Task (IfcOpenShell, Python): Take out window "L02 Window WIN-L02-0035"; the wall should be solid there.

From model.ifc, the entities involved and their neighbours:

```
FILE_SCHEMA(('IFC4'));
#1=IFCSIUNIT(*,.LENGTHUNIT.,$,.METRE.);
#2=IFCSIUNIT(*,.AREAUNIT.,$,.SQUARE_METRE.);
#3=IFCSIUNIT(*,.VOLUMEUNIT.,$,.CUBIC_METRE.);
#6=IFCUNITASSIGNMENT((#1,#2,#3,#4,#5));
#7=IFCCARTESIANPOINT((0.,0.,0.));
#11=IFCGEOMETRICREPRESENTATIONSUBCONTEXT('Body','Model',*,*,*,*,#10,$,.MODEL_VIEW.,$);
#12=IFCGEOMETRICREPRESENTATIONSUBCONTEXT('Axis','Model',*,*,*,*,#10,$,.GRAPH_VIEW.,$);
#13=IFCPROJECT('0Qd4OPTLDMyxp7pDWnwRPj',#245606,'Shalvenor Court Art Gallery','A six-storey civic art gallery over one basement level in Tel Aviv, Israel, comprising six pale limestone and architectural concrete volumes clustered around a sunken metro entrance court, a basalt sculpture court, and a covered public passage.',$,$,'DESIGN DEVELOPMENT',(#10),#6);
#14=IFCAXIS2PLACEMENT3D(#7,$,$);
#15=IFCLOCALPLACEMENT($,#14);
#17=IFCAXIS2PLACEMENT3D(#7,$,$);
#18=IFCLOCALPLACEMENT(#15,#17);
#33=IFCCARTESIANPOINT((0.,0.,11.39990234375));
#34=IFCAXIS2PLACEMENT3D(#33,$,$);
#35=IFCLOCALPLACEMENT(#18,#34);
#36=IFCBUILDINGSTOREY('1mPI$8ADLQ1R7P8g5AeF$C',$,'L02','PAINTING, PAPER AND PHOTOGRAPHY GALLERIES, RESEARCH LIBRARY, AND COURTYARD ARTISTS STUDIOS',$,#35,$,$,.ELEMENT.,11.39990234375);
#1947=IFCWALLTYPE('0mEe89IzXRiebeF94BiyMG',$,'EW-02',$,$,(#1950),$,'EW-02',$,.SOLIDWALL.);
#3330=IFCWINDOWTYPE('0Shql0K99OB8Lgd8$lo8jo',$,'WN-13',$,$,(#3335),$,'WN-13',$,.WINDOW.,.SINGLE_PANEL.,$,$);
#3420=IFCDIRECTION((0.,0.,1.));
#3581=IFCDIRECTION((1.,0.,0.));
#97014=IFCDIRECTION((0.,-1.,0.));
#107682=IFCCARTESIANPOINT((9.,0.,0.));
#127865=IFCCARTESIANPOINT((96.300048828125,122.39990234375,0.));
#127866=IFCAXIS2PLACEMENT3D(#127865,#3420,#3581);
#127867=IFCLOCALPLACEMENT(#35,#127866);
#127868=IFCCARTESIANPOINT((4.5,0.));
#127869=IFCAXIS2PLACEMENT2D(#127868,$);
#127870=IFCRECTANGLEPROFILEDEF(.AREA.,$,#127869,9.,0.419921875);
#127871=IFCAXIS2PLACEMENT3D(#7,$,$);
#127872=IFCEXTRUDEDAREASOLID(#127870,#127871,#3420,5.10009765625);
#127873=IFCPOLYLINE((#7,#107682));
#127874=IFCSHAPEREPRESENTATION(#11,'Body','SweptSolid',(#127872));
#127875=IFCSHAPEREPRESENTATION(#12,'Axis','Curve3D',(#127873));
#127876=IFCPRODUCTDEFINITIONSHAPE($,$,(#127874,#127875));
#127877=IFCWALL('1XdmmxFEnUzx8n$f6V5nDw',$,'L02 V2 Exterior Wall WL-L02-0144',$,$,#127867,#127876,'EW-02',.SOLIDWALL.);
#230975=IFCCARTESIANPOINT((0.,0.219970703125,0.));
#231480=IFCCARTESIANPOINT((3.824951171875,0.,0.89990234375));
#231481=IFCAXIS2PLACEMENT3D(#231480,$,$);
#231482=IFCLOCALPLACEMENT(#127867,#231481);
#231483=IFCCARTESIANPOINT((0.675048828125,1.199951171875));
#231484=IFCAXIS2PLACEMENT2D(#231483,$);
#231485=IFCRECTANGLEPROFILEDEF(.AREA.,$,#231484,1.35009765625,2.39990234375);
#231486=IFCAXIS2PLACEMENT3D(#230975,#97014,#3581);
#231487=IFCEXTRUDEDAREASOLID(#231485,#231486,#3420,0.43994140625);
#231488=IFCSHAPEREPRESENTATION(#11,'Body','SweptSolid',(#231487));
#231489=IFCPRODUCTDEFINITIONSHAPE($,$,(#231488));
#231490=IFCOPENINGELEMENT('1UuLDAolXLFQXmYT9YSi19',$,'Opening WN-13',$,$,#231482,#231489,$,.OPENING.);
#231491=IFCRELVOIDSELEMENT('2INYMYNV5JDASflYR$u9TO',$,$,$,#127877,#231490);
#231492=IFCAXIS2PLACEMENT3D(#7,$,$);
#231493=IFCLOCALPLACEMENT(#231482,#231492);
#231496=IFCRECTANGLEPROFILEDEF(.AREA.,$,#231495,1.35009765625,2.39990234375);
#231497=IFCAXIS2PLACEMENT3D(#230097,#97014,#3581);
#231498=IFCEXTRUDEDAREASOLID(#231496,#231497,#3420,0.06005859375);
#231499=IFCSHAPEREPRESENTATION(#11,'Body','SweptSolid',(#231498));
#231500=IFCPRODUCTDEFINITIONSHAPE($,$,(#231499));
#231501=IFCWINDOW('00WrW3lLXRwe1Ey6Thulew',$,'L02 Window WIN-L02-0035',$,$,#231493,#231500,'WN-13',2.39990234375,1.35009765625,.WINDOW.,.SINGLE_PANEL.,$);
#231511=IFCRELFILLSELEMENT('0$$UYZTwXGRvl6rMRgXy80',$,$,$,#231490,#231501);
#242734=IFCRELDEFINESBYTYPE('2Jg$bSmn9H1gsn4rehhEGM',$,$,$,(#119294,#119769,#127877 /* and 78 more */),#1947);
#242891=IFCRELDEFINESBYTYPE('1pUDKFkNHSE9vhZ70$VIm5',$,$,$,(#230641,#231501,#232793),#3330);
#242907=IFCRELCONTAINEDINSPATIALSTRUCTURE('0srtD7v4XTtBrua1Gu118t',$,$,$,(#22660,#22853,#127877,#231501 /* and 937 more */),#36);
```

```python
import ifcopenshell
import ifcopenshell.api.feature
import ifcopenshell.api.root
import ifcopenshell.geom
import ifcopenshell.util.shape

model = ifcopenshell.open("model.ifc")
settings = ifcopenshell.geom.settings()


def volume(element):
    """Net volume in cubic metres, openings subtracted."""
    shape = ifcopenshell.geom.create_shape(settings, element)
    return ifcopenshell.util.shape.get_volume(shape.geometry)


window = model.by_guid("00WrW3lLXRwe1Ey6Thulew")
opening = window.FillsVoids[0].RelatingOpeningElement
wall = opening.VoidsElements[0].RelatingBuildingElement
before = volume(wall)

ifcopenshell.api.root.remove_product(model, product=window)
ifcopenshell.api.feature.remove_feature(model, feature=opening)

after = volume(wall)

print(f"wall volume {before:.3f} -> {after:.3f} m3")

model.write("model_edited.ifc")
```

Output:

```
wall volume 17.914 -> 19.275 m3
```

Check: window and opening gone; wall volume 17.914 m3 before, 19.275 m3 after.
